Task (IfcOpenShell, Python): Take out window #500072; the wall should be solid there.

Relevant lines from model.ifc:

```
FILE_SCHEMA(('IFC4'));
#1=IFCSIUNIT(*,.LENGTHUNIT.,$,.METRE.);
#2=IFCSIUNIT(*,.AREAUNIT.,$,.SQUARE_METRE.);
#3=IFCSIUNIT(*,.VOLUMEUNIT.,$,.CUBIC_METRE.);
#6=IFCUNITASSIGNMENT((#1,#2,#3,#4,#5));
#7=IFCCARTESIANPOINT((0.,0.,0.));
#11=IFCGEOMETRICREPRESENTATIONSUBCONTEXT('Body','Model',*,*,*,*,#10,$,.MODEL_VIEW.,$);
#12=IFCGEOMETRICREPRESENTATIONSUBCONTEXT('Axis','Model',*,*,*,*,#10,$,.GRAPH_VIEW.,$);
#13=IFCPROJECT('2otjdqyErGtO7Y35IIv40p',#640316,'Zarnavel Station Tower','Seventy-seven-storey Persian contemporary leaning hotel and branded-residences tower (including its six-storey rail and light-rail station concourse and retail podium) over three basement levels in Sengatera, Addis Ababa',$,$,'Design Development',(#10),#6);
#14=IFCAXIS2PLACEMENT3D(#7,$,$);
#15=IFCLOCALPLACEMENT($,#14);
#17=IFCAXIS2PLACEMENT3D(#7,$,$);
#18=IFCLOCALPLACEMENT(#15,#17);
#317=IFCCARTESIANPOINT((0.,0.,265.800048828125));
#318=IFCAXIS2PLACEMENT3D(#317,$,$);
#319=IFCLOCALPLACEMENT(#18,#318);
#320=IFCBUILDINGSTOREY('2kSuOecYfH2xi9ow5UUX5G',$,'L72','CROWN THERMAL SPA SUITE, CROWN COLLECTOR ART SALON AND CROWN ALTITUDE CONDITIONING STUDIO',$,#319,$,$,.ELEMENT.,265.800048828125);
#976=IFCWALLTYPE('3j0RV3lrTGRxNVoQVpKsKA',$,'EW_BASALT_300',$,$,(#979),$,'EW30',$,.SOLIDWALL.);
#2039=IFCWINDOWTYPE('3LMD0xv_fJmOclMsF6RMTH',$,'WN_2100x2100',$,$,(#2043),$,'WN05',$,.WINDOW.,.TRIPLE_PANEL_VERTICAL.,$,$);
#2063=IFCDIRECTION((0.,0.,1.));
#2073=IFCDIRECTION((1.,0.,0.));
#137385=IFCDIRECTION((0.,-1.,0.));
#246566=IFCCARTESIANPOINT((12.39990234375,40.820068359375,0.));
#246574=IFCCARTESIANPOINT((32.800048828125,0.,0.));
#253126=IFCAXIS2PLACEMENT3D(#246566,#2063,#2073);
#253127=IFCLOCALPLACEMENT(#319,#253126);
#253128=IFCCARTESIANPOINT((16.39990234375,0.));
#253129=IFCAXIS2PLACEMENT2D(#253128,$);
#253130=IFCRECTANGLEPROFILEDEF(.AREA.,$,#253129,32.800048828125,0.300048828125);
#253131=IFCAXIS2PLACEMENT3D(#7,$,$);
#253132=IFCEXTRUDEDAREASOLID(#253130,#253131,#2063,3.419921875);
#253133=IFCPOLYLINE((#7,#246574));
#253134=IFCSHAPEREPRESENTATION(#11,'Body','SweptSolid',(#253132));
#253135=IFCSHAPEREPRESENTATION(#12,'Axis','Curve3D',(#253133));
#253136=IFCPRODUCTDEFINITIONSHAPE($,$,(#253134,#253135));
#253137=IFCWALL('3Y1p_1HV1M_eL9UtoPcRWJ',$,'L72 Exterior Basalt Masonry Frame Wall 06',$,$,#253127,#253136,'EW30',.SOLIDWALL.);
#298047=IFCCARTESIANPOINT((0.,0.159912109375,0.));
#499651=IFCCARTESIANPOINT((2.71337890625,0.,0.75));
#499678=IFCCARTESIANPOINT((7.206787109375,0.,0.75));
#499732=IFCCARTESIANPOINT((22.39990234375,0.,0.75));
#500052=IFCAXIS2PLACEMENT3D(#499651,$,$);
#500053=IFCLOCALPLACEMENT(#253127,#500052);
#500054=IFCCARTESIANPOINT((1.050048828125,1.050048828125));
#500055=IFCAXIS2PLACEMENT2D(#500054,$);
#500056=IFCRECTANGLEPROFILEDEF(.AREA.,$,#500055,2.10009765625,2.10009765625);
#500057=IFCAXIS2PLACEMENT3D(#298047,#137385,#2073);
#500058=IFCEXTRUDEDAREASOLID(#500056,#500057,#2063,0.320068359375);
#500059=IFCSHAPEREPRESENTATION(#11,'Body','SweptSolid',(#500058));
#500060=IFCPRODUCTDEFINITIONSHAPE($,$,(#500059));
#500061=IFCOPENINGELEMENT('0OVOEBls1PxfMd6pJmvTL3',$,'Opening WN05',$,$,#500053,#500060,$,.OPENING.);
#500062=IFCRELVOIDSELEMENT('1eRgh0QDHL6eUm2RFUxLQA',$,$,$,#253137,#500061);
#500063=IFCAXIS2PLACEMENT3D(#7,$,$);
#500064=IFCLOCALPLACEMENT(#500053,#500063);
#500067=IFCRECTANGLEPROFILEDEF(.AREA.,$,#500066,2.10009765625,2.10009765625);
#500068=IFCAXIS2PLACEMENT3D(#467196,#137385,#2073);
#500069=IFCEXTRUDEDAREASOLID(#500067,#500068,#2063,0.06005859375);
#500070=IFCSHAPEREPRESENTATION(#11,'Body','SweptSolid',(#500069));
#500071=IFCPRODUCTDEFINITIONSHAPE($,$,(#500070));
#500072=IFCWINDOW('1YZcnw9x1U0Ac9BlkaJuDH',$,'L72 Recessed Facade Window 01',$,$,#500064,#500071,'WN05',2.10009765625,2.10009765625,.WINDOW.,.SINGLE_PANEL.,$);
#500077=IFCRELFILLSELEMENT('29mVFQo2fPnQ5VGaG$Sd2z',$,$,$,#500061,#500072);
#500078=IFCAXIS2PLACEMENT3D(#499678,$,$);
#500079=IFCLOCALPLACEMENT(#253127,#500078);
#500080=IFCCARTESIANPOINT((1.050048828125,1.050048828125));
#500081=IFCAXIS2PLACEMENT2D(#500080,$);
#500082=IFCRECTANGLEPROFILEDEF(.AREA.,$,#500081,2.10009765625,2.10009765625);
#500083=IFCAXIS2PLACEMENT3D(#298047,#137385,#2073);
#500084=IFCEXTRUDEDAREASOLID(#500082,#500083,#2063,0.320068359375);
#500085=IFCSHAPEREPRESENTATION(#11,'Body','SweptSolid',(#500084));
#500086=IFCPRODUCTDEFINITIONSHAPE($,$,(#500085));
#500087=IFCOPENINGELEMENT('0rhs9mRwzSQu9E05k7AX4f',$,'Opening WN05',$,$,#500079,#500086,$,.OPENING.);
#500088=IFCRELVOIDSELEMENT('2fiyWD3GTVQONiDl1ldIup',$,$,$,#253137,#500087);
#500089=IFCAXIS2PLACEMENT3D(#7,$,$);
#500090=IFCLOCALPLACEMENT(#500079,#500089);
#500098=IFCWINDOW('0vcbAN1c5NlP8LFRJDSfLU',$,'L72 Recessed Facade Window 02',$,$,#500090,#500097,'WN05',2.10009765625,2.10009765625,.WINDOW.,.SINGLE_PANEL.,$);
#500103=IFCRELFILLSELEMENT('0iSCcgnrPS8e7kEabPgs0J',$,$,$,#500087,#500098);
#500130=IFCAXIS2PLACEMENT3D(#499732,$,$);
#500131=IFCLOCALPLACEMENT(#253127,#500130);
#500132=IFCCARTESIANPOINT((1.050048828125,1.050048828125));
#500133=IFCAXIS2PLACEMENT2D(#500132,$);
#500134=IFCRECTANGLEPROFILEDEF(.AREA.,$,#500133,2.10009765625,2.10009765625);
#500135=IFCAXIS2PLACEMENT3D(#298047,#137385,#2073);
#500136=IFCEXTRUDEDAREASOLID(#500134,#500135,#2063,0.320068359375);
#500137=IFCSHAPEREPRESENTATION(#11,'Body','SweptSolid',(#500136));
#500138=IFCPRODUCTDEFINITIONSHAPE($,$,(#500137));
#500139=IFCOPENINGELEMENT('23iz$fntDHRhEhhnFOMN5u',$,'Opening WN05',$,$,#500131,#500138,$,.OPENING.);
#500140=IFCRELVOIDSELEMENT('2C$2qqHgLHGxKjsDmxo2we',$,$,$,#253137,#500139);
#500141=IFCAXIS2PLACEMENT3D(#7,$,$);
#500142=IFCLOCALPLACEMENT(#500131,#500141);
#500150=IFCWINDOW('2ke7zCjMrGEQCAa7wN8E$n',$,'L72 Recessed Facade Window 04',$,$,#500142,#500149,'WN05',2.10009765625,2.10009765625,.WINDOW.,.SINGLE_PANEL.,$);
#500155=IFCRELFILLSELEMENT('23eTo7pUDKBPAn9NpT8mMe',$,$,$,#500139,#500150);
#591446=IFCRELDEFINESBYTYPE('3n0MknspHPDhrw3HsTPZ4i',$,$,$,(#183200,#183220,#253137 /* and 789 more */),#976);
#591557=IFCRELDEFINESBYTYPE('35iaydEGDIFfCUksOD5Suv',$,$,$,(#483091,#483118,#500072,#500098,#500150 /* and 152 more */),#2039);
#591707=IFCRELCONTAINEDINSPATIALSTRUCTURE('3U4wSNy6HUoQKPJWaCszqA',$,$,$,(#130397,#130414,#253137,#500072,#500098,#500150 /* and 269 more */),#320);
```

```python
import ifcopenshell
import ifcopenshell.api.feature
import ifcopenshell.api.root
import ifcopenshell.geom
import ifcopenshell.util.shape

model = ifcopenshell.open("model.ifc")
settings = ifcopenshell.geom.settings()


def volume(element):
    """Net volume in cubic metres, openings subtracted."""
    shape = ifcopenshell.geom.create_shape(settings, element)
    return ifcopenshell.util.shape.get_volume(shape.geometry)


window = model.by_guid("1YZcnw9x1U0Ac9BlkaJuDH")
opening = window.FillsVoids[0].RelatingOpeningElement
wall = opening.VoidsElements[0].RelatingBuildingElement
before = volume(wall)

ifcopenshell.api.root.remove_product(model, product=window)
ifcopenshell.api.feature.remove_feature(model, feature=opening)

after = volume(wall)

print(f"wall volume {before:.3f} -> {after:.3f} m3")

model.write("model_edited.ifc")
```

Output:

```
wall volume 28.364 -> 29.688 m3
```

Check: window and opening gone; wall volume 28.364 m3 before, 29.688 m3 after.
